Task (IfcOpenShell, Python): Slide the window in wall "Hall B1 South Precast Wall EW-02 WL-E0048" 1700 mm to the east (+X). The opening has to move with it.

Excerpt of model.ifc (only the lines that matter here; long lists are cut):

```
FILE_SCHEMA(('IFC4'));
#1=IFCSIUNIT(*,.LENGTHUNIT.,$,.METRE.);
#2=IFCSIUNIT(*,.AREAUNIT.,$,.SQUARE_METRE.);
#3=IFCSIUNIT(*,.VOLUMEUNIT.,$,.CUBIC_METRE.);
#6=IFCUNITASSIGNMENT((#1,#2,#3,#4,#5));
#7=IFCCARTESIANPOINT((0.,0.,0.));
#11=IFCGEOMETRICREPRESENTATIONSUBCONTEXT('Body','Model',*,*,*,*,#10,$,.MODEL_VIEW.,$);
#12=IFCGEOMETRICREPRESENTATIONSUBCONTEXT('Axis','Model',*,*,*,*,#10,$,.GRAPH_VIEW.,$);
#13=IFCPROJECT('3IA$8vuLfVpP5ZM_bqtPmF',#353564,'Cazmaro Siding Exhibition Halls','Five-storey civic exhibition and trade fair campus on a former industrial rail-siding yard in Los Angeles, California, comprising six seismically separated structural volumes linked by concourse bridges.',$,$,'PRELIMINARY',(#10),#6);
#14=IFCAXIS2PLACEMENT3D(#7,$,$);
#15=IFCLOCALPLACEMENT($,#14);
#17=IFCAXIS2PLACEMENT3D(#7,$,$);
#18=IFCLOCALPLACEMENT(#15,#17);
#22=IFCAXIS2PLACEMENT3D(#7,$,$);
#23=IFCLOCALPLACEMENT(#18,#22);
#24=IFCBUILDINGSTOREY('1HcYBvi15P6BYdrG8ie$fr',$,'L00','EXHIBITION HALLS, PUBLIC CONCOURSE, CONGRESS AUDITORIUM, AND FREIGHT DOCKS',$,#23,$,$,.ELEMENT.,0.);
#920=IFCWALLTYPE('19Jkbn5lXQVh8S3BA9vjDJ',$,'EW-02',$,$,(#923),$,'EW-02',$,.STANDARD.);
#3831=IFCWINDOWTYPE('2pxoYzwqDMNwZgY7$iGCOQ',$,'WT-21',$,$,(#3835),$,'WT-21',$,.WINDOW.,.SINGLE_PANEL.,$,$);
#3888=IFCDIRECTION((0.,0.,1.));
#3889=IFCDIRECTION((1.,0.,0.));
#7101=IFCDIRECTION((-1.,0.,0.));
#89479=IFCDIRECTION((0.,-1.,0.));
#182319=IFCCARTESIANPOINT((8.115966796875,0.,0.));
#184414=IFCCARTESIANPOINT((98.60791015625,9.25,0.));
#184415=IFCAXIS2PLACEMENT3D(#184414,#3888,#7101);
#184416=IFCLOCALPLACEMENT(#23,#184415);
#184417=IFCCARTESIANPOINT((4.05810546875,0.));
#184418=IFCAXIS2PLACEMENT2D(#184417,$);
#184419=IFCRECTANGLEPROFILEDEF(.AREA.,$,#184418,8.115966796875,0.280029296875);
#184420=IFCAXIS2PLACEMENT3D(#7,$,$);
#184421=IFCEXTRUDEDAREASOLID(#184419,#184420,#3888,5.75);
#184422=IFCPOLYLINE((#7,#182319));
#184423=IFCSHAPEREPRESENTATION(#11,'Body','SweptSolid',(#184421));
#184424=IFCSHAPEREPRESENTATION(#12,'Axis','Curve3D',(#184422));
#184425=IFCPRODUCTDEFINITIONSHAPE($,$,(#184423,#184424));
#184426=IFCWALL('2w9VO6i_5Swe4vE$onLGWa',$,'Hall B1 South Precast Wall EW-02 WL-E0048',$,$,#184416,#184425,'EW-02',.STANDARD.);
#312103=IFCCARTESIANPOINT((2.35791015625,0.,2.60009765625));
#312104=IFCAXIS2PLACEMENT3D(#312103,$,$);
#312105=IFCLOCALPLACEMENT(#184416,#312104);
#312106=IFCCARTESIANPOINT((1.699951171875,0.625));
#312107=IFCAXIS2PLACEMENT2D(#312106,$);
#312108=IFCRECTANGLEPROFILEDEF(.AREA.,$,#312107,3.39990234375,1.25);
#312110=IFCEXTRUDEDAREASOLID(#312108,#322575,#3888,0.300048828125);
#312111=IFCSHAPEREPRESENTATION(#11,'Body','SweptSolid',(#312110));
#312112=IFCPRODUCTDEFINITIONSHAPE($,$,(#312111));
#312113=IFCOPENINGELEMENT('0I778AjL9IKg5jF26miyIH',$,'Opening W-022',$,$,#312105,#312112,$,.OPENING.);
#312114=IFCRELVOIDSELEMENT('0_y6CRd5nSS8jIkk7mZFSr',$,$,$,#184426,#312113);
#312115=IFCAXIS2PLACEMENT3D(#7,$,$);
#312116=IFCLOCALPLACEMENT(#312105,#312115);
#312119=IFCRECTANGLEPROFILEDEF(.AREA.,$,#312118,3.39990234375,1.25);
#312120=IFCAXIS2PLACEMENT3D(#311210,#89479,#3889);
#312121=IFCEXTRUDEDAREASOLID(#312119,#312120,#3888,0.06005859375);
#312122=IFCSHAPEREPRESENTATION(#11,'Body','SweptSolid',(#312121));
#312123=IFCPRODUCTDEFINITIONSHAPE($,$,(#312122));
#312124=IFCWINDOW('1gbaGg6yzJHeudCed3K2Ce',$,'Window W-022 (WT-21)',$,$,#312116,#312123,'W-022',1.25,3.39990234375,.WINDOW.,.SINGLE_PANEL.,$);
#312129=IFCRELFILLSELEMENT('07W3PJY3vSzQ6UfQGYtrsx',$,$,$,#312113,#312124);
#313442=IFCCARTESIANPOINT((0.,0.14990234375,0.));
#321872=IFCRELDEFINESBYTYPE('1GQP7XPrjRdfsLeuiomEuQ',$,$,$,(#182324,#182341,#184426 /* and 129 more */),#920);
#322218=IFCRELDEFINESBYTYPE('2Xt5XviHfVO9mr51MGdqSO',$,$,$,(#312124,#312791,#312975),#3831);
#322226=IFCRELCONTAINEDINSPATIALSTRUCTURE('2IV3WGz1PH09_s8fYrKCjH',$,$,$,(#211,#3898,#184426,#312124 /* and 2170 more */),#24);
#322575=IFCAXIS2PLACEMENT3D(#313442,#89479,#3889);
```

```python
import ifcopenshell
import ifcopenshell.api.geometry
import ifcopenshell.util.placement

model = ifcopenshell.open("model.ifc")

window = model.by_guid("1gbaGg6yzJHeudCed3K2Ce")
opening = window.FillsVoids[0].RelatingOpeningElement
wall = opening.VoidsElements[0].RelatingBuildingElement

wall_matrix = ifcopenshell.util.placement.get_local_placement(wall.ObjectPlacement)
shift = wall_matrix[:3, 0] * -1.7
before = ifcopenshell.util.placement.get_local_placement(window.ObjectPlacement)[:3, 3].copy()

# The window is placed relative to its opening, so it follows when the opening moves.
matrix = ifcopenshell.util.placement.get_local_placement(opening.ObjectPlacement)
matrix[:3, 3] += shift
ifcopenshell.api.geometry.edit_object_placement(
    model, product=opening, matrix=matrix, is_si=False, should_transform_children=True
)

after = ifcopenshell.util.placement.get_local_placement(window.ObjectPlacement)[:3, 3]
print("window moved by", (after - before).round(3) + 0.0)

model.write("model_v2.ifc")
```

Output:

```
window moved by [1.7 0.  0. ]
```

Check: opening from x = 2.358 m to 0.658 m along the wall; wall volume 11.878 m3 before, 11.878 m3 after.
